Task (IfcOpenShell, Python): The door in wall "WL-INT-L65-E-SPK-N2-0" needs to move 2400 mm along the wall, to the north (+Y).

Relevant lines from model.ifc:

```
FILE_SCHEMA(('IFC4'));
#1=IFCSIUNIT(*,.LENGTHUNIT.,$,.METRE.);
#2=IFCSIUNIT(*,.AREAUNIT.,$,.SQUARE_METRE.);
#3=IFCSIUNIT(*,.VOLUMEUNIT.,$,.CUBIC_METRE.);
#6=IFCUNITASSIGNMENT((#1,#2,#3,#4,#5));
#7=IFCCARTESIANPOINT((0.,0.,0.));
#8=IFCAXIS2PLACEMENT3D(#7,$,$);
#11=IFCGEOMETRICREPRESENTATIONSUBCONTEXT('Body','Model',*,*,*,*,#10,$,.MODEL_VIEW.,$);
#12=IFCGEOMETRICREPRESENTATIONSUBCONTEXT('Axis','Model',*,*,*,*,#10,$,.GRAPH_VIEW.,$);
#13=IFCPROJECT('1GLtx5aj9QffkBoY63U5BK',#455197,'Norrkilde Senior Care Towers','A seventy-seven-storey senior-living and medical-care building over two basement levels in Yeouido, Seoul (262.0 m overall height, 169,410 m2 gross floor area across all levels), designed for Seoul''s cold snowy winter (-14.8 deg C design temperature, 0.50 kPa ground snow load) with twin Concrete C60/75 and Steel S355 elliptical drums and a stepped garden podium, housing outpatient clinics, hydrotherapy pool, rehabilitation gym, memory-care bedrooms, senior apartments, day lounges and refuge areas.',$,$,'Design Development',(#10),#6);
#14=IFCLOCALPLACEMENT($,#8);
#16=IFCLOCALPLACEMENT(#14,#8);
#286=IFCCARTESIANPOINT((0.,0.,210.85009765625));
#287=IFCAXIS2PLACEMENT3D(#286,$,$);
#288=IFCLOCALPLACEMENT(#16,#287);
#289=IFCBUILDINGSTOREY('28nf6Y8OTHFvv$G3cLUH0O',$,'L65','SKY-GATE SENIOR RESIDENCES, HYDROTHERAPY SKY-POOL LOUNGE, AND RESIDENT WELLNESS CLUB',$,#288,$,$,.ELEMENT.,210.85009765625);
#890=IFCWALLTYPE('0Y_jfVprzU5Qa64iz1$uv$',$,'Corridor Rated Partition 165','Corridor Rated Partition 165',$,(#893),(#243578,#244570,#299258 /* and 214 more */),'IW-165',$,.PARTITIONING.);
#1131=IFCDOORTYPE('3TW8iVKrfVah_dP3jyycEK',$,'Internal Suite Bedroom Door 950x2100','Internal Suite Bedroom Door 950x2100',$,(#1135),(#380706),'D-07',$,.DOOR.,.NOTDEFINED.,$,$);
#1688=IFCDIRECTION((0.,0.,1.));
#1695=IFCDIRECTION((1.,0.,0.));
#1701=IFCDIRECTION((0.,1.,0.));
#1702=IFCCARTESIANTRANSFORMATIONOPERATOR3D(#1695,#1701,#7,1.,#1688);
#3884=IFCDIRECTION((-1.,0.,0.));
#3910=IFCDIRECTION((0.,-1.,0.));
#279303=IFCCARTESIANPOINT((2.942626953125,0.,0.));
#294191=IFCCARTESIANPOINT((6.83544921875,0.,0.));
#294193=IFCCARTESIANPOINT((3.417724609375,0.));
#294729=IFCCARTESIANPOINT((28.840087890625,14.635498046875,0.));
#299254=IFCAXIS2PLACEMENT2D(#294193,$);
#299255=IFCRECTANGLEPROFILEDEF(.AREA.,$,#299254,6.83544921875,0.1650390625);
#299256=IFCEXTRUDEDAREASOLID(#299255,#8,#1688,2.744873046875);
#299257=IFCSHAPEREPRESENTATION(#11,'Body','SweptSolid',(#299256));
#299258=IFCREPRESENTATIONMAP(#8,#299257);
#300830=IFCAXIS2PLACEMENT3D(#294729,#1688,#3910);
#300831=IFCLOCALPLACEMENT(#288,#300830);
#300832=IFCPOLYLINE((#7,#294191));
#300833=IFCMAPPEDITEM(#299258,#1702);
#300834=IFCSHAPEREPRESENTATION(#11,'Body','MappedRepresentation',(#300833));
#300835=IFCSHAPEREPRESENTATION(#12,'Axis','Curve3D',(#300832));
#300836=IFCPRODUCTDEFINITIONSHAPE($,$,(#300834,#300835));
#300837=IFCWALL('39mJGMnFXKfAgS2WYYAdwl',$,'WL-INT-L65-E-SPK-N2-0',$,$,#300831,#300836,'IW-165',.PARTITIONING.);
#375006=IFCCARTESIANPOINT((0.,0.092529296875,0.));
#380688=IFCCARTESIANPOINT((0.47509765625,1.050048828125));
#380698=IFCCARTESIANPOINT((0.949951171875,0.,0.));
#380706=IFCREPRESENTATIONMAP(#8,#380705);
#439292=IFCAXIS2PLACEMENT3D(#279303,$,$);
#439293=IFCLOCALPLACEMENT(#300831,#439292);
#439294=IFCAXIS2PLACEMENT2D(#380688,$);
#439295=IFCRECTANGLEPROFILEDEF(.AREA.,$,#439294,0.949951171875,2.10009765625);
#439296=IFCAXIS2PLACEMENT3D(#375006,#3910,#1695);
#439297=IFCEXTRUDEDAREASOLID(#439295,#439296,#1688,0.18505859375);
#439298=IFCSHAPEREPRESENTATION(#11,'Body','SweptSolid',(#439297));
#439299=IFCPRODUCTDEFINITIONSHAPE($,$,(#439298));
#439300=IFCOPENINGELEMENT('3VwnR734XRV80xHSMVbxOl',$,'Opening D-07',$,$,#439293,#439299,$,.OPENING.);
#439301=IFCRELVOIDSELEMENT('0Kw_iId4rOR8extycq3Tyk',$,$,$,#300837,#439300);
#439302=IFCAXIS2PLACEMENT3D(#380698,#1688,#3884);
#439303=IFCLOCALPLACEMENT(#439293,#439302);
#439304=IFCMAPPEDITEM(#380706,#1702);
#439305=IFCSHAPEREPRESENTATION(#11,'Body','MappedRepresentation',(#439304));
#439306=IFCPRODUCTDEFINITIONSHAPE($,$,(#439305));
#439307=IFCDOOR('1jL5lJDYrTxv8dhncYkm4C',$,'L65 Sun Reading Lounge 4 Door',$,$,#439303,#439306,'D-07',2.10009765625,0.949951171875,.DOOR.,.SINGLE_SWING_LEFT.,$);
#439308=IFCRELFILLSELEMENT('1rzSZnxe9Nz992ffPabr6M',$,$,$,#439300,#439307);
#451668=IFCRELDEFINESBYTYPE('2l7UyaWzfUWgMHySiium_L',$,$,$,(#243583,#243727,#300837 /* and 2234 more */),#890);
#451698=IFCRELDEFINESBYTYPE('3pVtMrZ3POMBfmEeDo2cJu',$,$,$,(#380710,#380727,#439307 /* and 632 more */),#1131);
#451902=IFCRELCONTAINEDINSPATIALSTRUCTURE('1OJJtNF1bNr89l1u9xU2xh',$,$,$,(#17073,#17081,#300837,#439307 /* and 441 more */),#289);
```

```python
import ifcopenshell
import ifcopenshell.api.geometry
import ifcopenshell.util.placement

model = ifcopenshell.open("model.ifc")

door = model.by_guid("1jL5lJDYrTxv8dhncYkm4C")
opening = door.FillsVoids[0].RelatingOpeningElement
wall = opening.VoidsElements[0].RelatingBuildingElement

wall_matrix = ifcopenshell.util.placement.get_local_placement(wall.ObjectPlacement)
shift = wall_matrix[:3, 0] * -2.4
before = ifcopenshell.util.placement.get_local_placement(door.ObjectPlacement)[:3, 3].copy()

# The door is placed relative to its opening, so it follows when the opening moves.
matrix = ifcopenshell.util.placement.get_local_placement(opening.ObjectPlacement)
matrix[:3, 3] += shift
ifcopenshell.api.geometry.edit_object_placement(
    model, product=opening, matrix=matrix, is_si=False, should_transform_children=True
)

after = ifcopenshell.util.placement.get_local_placement(door.ObjectPlacement)[:3, 3]
print("door moved by", (after - before).round(3) + 0.0)

model.write("model_rev.ifc")
```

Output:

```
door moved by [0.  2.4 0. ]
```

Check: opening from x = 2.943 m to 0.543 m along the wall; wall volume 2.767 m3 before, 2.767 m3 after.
